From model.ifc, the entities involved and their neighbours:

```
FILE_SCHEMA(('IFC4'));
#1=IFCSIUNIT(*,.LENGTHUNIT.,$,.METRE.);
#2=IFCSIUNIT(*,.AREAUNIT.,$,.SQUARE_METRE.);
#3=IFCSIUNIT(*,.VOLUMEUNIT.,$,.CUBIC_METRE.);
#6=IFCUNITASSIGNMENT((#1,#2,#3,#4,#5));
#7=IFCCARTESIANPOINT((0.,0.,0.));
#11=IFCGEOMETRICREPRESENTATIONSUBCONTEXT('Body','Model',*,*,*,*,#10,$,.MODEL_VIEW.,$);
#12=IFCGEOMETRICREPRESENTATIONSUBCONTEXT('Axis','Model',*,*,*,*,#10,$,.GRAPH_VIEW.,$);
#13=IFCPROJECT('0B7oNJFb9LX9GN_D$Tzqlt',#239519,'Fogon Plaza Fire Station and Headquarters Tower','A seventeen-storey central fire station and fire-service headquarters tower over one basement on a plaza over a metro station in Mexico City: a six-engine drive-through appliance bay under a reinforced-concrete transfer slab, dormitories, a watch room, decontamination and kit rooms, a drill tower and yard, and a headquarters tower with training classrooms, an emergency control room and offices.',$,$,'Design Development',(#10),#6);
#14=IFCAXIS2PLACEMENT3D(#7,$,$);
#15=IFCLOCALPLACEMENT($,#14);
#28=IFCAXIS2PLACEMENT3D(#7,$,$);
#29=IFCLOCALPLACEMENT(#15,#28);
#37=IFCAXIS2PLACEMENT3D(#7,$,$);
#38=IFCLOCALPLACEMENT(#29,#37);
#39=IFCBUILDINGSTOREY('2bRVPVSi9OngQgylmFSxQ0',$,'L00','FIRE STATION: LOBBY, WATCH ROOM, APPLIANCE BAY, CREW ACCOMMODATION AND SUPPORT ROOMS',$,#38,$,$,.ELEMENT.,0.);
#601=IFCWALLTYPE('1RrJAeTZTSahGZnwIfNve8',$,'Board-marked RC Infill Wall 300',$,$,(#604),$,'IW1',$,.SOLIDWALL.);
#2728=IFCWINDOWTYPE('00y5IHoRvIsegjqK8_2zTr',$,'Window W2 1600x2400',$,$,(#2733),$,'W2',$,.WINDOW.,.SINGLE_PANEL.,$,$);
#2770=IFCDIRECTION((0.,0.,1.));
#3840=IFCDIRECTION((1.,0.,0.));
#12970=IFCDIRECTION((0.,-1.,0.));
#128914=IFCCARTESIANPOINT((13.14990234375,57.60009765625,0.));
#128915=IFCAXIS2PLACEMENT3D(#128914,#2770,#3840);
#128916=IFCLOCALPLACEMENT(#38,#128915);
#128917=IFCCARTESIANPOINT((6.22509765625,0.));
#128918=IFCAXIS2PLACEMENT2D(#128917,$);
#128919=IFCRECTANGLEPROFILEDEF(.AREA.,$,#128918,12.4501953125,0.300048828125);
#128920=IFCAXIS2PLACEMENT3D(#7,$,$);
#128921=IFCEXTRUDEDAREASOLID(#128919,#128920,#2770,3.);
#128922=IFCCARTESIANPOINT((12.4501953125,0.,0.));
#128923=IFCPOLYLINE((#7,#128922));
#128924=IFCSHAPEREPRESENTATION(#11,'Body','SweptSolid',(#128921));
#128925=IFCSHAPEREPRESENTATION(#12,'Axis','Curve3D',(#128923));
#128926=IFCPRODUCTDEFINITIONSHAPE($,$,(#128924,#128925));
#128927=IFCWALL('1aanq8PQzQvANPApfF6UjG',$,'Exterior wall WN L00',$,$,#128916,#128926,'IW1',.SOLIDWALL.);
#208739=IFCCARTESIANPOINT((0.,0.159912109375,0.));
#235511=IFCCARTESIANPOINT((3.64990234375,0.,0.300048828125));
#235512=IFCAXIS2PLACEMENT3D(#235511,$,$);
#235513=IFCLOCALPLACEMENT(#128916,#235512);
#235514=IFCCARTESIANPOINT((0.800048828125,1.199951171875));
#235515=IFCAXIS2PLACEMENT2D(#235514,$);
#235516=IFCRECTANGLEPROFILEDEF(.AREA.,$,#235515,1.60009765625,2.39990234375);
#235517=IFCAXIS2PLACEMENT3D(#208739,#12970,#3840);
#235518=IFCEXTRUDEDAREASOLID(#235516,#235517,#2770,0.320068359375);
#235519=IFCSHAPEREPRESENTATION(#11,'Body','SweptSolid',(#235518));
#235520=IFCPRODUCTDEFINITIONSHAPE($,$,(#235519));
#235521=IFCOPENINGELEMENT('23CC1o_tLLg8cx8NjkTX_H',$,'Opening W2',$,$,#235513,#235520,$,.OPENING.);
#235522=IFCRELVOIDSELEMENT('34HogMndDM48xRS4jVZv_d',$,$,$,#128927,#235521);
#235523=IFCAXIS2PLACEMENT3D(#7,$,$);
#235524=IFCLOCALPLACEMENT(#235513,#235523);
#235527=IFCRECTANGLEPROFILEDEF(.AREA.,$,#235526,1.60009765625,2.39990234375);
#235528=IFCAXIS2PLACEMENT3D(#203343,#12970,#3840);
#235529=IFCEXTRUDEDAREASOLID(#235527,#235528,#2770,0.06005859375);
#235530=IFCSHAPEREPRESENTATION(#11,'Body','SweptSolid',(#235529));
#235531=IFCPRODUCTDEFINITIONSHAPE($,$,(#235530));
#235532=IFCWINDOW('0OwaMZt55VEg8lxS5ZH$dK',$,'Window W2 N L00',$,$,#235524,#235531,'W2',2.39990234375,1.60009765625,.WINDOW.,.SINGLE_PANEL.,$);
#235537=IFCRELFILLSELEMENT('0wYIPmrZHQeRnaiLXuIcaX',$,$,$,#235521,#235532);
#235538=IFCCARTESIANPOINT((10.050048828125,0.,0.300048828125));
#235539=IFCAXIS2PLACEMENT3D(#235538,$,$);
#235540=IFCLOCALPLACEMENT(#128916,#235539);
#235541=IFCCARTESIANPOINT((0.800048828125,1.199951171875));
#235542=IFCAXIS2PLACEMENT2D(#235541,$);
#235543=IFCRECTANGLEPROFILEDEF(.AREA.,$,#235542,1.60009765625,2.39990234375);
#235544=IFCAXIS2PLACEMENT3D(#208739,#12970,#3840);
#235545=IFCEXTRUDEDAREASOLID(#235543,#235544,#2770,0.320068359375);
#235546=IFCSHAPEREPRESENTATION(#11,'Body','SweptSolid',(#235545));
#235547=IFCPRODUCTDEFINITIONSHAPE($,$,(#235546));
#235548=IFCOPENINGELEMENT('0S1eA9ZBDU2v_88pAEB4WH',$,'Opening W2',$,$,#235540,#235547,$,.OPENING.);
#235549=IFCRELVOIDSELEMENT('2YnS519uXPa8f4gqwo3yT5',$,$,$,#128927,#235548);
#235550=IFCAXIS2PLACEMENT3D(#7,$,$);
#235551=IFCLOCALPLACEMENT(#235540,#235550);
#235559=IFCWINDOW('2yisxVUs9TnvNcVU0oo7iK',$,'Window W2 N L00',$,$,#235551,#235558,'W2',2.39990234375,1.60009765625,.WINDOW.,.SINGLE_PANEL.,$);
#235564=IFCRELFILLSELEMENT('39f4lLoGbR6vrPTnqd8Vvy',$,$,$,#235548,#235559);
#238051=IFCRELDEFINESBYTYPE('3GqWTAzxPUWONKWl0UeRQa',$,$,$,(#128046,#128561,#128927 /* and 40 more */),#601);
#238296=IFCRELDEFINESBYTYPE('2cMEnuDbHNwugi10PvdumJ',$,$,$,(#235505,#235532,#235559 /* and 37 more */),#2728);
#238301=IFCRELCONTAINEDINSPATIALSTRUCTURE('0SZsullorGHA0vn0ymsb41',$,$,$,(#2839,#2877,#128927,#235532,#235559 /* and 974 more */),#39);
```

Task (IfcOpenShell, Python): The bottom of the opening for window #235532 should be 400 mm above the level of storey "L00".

```python
import numpy as np
import ifcopenshell
import ifcopenshell.api.geometry
import ifcopenshell.geom
import ifcopenshell.util.element
import ifcopenshell.util.placement
import ifcopenshell.util.shape
import ifcopenshell.util.unit

model = ifcopenshell.open("model.ifc")
unit_scale = ifcopenshell.util.unit.calculate_unit_scale(model)

window = model.by_guid("0OwaMZt55VEg8lxS5ZH$dK")
opening = window.FillsVoids[0].RelatingOpeningElement
storey = ifcopenshell.util.element.get_container(window, ifc_class="IfcBuildingStorey")
level = ifcopenshell.util.placement.get_local_placement(storey.ObjectPlacement)[2, 3]

# The opening's origin need not be at the sill, so measure its lowest point.
shape = ifcopenshell.geom.create_shape(ifcopenshell.geom.settings(), opening)
bottom = ifcopenshell.util.shape.get_shape_bottom_elevation(shape, shape.geometry) / unit_scale
dz = level + 0.4 / unit_scale - bottom

shift = np.array([0.0, 0.0, dz])
# The window is placed relative to its opening, so it follows when the opening moves.
matrix = ifcopenshell.util.placement.get_local_placement(opening.ObjectPlacement)
matrix[:3, 3] += shift
ifcopenshell.api.geometry.edit_object_placement(
    model, product=opening, matrix=matrix, is_si=False, should_transform_children=True
)

print(f"moved by {dz * unit_scale:+.3f} m")

model.write("model_edited.ifc")
```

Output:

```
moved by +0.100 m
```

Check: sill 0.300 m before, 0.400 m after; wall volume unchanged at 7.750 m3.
